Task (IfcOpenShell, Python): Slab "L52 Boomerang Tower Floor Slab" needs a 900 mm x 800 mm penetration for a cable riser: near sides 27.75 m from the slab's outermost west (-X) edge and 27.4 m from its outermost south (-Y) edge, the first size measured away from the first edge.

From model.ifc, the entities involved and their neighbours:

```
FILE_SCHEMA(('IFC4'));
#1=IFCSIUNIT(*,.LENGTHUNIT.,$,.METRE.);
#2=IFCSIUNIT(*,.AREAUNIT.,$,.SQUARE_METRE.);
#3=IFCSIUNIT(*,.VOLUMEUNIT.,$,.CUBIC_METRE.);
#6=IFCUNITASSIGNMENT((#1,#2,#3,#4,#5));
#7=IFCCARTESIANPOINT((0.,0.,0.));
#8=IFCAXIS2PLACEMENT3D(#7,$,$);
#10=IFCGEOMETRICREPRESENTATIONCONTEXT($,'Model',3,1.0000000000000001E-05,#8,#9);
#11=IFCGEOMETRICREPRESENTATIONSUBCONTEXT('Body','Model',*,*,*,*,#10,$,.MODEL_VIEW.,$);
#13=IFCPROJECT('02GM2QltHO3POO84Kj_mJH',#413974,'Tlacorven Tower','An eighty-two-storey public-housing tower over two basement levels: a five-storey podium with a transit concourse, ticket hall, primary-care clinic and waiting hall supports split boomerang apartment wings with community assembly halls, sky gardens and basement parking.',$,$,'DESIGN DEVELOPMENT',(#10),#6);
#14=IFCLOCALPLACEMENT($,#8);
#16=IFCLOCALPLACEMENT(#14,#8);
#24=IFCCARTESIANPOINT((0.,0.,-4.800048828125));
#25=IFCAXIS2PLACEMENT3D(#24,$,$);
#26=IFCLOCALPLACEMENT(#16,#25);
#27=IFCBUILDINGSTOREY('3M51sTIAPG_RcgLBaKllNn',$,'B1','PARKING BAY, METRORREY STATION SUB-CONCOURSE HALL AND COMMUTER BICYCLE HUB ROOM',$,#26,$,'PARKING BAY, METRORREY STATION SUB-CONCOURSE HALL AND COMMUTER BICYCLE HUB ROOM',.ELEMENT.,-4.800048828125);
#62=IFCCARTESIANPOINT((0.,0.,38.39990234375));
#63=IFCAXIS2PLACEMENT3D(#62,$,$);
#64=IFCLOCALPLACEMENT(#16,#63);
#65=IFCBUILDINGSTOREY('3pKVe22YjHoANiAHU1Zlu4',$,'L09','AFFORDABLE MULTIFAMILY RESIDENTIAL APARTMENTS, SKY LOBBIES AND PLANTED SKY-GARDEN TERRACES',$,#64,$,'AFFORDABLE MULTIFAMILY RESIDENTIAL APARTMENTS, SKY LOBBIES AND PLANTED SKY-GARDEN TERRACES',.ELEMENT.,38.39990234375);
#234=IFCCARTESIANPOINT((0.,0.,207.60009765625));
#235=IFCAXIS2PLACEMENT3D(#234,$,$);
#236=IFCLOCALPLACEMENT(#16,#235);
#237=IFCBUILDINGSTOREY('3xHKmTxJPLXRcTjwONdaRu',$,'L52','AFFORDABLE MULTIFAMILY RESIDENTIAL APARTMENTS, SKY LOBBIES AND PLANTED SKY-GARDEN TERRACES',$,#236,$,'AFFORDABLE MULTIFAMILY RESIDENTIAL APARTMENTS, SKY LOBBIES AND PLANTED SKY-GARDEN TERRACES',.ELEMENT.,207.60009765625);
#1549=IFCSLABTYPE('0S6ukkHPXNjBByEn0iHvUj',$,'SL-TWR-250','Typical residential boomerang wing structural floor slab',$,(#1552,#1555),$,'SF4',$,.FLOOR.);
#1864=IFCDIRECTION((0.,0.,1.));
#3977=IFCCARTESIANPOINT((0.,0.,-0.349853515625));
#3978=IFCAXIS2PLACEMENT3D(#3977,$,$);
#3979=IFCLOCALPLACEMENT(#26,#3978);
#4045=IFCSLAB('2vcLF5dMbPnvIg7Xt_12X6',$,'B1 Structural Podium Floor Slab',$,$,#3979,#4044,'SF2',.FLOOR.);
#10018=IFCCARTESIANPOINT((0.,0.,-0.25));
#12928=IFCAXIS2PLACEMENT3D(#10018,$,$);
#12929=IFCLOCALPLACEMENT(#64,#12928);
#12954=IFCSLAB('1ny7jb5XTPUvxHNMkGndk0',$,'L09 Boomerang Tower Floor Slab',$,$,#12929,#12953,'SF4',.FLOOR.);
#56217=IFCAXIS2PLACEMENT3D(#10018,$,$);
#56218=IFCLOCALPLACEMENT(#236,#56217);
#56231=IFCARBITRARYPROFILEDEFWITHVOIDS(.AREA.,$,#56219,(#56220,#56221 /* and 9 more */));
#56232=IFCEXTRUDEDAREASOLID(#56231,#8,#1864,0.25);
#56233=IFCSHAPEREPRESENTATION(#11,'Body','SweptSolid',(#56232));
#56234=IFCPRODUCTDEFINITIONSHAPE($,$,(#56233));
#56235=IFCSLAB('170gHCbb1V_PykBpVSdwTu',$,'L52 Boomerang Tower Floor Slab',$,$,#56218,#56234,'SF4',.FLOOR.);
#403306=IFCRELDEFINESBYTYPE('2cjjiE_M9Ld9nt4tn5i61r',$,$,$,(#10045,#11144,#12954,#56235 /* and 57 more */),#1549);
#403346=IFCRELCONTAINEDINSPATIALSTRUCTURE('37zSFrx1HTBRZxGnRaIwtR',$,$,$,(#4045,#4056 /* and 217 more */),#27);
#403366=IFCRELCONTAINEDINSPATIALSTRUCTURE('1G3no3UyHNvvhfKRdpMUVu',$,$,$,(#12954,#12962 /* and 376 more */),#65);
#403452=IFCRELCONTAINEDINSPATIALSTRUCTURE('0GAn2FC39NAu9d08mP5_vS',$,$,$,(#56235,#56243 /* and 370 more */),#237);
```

```python
import numpy as np
import ifcopenshell
import ifcopenshell.api.feature
import ifcopenshell.api.geometry
import ifcopenshell.api.root
import ifcopenshell.geom
import ifcopenshell.util.placement
import ifcopenshell.util.representation
import ifcopenshell.util.shape
import ifcopenshell.util.unit

model = ifcopenshell.open("model.ifc")
unit_scale = ifcopenshell.util.unit.calculate_unit_scale(model)
settings = ifcopenshell.geom.settings()


def volume(element):
    """Net volume in cubic metres, openings subtracted."""
    shape = ifcopenshell.geom.create_shape(settings, element)
    return ifcopenshell.util.shape.get_volume(shape.geometry)


slab = model.by_id(56235)
before = volume(slab)

# Extent in the slab's own axes, in metres. The edges named are its -X and -Y sides.
slab_shape = ifcopenshell.geom.create_shape(settings, slab)
vertices = ifcopenshell.util.shape.get_vertices(slab_shape.geometry)
x_min, y_min, bottom = vertices.min(axis=0)
top = vertices[:, 2].max()

opening = ifcopenshell.api.root.create_entity(model, ifc_class="IfcOpeningElement", name="Cable riser opening", predefined_type="OPENING")
context = ifcopenshell.util.representation.get_context(model, "Model", "Body", "MODEL_VIEW")
width, depth = 0.9, 0.8
outline = [(0.0, 0.0), (width, 0.0), (width, depth), (0.0, depth), (0.0, 0.0)]
# Overshoot both faces by 50 mm so the cut is clean.
shape = ifcopenshell.api.geometry.add_slab_representation(
    model, context=context, depth=top - bottom + 0.1, polyline=outline
)
ifcopenshell.api.geometry.assign_representation(model, product=opening, representation=shape)

matrix = ifcopenshell.util.placement.get_local_placement(slab.ObjectPlacement)
matrix[:, 3] = matrix @ np.append(np.array([x_min + 27.75, y_min + 27.4, bottom - 0.05]) / unit_scale, 1.0)
ifcopenshell.api.geometry.edit_object_placement(model, product=opening, matrix=matrix, is_si=False)
ifcopenshell.api.feature.add_feature(model, feature=opening, element=slab)

after = volume(slab)

print(f"slab volume {before:.3f} -> {after:.3f} m3")

model.write("model_updated.ifc")
```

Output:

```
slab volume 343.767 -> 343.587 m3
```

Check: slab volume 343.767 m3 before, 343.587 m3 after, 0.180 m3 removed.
